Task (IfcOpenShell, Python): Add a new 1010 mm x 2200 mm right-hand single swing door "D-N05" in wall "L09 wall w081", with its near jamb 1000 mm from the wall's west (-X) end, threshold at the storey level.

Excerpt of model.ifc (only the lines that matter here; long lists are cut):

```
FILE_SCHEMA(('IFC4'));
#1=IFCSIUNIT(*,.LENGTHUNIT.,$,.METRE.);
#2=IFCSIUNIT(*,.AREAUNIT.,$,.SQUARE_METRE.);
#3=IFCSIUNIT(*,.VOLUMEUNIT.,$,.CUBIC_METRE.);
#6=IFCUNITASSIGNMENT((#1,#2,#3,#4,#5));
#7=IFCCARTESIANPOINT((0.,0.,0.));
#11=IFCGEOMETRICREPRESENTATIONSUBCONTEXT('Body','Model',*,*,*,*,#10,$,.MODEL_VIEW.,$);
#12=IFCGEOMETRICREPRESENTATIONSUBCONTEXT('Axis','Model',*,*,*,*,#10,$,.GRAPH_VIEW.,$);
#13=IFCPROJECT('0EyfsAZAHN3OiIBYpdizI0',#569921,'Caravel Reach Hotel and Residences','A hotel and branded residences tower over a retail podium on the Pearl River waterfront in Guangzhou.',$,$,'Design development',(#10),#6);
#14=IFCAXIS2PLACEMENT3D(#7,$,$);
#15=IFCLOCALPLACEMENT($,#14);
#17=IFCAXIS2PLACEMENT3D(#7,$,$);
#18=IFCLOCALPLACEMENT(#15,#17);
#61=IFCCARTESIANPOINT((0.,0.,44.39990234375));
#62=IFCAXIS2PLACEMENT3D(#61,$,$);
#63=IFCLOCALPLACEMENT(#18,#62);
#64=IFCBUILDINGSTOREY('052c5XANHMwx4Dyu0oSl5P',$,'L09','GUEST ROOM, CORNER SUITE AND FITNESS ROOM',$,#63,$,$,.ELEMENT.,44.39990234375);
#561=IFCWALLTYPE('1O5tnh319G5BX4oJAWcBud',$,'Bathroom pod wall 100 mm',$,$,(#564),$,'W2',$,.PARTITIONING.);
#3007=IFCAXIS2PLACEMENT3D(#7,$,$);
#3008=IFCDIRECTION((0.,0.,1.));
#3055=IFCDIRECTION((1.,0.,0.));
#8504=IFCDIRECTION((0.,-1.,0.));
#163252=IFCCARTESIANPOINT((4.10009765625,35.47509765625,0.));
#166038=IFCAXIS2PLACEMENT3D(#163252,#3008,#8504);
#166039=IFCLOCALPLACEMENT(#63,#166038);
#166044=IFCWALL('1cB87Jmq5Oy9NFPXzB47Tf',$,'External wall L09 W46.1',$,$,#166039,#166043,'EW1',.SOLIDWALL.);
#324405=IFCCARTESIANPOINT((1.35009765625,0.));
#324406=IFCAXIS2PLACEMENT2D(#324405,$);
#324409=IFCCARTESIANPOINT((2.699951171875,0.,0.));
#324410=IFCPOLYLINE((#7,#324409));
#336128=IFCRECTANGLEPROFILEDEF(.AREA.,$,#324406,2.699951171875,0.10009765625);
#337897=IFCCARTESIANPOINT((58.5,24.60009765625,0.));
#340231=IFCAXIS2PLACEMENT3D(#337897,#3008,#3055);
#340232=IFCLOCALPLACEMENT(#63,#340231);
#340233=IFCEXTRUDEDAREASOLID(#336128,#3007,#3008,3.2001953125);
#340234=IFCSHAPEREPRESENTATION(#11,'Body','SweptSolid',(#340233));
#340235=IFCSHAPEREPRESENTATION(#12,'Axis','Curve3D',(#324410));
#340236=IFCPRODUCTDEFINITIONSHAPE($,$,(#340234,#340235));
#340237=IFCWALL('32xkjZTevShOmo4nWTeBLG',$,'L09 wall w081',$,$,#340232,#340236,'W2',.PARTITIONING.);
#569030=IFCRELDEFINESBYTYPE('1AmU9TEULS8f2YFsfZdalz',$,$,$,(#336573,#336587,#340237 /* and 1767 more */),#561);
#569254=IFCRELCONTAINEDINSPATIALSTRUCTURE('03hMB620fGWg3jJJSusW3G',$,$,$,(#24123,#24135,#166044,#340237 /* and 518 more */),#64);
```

```python
import numpy as np
import ifcopenshell
import ifcopenshell.api.feature
import ifcopenshell.api.geometry
import ifcopenshell.api.root
import ifcopenshell.api.spatial
import ifcopenshell.geom
import ifcopenshell.util.element
import ifcopenshell.util.placement
import ifcopenshell.util.representation
import ifcopenshell.util.shape
import ifcopenshell.util.unit

model = ifcopenshell.open("model.ifc")
unit_scale = ifcopenshell.util.unit.calculate_unit_scale(model)
settings = ifcopenshell.geom.settings()


def volume(element):
    """Net volume in cubic metres, openings subtracted."""
    shape = ifcopenshell.geom.create_shape(settings, element)
    return ifcopenshell.util.shape.get_volume(shape.geometry)


wall = model.by_guid("32xkjZTevShOmo4nWTeBLG")
storey = ifcopenshell.util.element.get_container(wall, ifc_class="IfcBuildingStorey")
context = ifcopenshell.util.representation.get_context(model, "Model", "Body", "MODEL_VIEW")
before = volume(wall)

width, height, from_end, sill = 1.01, 2.2, 1, 0.0  # metres

# The wall runs along its own X axis, and the end named is its -X end.
wall_shape = ifcopenshell.geom.create_shape(settings, wall)
x, y, z = ifcopenshell.util.shape.get_vertices(wall_shape.geometry).T
start = x.min() + from_end
face, thickness = float(y.min()), float(y.max() - y.min())
wall_matrix = ifcopenshell.util.placement.get_local_placement(wall.ObjectPlacement)
level = ifcopenshell.util.placement.get_local_placement(storey.ObjectPlacement)[2, 3]


def in_wall(x, y):
    """Placement at x, y metres in the wall's axes, at sill height."""
    matrix = wall_matrix.copy()
    matrix[:, 3] = wall_matrix @ np.array([x / unit_scale, y / unit_scale, 0.0, 1.0])
    matrix[2, 3] = level + sill / unit_scale
    return matrix


# Opening: a box that overshoots both wall faces by 50 mm.
opening = ifcopenshell.api.root.create_entity(model, ifc_class="IfcOpeningElement", predefined_type="OPENING")
box = ifcopenshell.api.geometry.add_wall_representation(
    model, context=context, length=width, height=height, thickness=thickness + 0.1
)
ifcopenshell.api.geometry.assign_representation(model, product=opening, representation=box)
ifcopenshell.api.geometry.edit_object_placement(model, product=opening, matrix=in_wall(start, face - 0.05), is_si=False)
ifcopenshell.api.feature.add_feature(model, feature=opening, element=wall)

door = ifcopenshell.api.root.create_entity(model, ifc_class="IfcDoor", name="D-N05", predefined_type="DOOR")
door.OverallWidth, door.OverallHeight = width / unit_scale, height / unit_scale
door.OperationType = "SINGLE_SWING_RIGHT"
body = ifcopenshell.api.geometry.add_door_representation(
    model,
    context=context,
    overall_width=door.OverallWidth,
    overall_height=door.OverallHeight,
    operation_type="SINGLE_SWING_RIGHT",
    lining_properties={"LiningDepth": thickness / unit_scale, "ThresholdDepth": thickness / unit_scale},
)
ifcopenshell.api.geometry.assign_representation(model, product=door, representation=body)
ifcopenshell.api.spatial.assign_container(model, products=[door], relating_structure=storey)
ifcopenshell.api.feature.add_filling(model, opening=opening, element=door)

# The lining spans the wall, so the door starts at the wall face.
ifcopenshell.api.geometry.edit_object_placement(model, product=door, matrix=in_wall(start, face), is_si=False)

after = volume(wall)

print(f"wall volume {before:.3f} -> {after:.3f} m3")

model.write("model_edited.ifc")
```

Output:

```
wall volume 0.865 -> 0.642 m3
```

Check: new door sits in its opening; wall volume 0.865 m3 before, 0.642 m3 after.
